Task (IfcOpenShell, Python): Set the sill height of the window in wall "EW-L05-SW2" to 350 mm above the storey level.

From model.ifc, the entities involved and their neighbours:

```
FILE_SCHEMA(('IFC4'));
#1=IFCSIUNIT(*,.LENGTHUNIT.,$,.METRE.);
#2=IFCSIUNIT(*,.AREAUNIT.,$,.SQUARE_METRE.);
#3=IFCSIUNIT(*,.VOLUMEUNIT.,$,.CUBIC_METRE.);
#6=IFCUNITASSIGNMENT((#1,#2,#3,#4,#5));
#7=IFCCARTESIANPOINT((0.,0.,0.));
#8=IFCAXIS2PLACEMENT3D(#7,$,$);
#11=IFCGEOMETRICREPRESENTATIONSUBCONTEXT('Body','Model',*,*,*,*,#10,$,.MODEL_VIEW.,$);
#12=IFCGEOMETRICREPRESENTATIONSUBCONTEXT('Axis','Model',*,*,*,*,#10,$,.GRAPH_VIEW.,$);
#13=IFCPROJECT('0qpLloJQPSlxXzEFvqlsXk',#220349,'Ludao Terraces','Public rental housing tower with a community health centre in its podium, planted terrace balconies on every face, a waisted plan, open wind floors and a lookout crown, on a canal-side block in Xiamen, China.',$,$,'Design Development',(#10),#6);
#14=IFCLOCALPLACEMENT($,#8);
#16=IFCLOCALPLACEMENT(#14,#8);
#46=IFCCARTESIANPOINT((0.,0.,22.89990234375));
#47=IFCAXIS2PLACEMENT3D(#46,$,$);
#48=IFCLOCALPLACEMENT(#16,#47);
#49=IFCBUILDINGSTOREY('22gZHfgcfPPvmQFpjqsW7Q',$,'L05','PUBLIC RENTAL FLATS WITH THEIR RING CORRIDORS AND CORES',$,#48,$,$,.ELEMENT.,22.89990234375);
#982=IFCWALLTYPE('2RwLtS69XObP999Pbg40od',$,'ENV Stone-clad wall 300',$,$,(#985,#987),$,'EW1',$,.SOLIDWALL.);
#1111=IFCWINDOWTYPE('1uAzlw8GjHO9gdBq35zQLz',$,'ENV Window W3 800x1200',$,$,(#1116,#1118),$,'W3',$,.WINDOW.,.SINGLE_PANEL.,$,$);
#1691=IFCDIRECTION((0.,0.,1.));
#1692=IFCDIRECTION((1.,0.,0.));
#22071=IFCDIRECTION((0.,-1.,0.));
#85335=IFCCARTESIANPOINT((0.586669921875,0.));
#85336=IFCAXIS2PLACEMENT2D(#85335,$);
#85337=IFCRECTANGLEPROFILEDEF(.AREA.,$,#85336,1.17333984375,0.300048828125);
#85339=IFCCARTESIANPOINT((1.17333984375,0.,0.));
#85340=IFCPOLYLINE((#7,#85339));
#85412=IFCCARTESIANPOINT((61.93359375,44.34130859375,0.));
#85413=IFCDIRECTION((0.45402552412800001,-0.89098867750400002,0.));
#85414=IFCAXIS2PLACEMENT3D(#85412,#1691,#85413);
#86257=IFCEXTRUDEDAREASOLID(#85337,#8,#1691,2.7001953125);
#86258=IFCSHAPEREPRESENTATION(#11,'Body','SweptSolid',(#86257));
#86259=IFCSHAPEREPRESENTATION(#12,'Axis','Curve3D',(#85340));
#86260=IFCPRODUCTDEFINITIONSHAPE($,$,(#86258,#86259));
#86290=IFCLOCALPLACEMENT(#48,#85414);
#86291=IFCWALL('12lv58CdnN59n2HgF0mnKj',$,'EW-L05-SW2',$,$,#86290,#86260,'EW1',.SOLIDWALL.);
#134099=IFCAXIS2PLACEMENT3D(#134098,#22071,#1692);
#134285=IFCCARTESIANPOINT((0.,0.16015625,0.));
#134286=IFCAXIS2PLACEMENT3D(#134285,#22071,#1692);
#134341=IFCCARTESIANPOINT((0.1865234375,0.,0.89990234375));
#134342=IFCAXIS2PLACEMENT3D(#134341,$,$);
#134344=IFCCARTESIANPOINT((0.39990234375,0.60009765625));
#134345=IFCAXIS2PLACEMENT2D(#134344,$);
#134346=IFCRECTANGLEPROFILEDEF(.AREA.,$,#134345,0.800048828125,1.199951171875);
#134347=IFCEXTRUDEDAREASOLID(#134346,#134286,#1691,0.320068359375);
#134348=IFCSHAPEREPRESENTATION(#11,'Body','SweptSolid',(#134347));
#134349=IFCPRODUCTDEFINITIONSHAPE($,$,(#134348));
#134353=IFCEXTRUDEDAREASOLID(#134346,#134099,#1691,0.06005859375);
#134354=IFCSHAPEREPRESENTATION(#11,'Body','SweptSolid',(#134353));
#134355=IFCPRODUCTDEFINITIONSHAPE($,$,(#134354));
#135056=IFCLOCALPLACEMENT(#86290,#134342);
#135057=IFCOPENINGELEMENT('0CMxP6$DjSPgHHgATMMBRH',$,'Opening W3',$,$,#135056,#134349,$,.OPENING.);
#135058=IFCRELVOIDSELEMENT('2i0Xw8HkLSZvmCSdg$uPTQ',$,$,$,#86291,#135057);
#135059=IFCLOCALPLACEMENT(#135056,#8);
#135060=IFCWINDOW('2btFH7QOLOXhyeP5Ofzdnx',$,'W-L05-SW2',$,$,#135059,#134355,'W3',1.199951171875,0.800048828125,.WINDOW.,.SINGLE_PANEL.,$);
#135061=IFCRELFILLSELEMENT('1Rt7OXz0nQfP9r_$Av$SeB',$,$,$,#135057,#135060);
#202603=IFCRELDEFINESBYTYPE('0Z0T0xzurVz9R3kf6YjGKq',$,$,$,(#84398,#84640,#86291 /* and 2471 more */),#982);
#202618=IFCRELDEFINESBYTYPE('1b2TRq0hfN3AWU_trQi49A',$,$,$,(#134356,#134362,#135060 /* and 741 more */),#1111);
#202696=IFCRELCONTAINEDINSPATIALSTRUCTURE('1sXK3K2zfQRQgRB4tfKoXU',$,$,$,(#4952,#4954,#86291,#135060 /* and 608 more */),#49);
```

```python
import numpy as np
import ifcopenshell
import ifcopenshell.api.geometry
import ifcopenshell.geom
import ifcopenshell.util.element
import ifcopenshell.util.placement
import ifcopenshell.util.shape
import ifcopenshell.util.unit

model = ifcopenshell.open("model.ifc")
unit_scale = ifcopenshell.util.unit.calculate_unit_scale(model)

window = model.by_id(135060)
opening = window.FillsVoids[0].RelatingOpeningElement
storey = ifcopenshell.util.element.get_container(window, ifc_class="IfcBuildingStorey")
level = ifcopenshell.util.placement.get_local_placement(storey.ObjectPlacement)[2, 3]

# The opening's origin need not be at the sill, so measure its lowest point.
shape = ifcopenshell.geom.create_shape(ifcopenshell.geom.settings(), opening)
bottom = ifcopenshell.util.shape.get_shape_bottom_elevation(shape, shape.geometry) / unit_scale
dz = level + 0.35 - bottom

shift = np.array([0.0, 0.0, dz])
# The window is placed relative to its opening, so it follows when the opening moves.
matrix = ifcopenshell.util.placement.get_local_placement(opening.ObjectPlacement)
matrix[:3, 3] += shift
ifcopenshell.api.geometry.edit_object_placement(
    model, product=opening, matrix=matrix, is_si=False, should_transform_children=True
)

print(f"moved by {dz * unit_scale:+.3f} m")

model.write("model_edited.ifc")
```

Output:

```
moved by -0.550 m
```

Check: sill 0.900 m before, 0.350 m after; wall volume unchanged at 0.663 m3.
